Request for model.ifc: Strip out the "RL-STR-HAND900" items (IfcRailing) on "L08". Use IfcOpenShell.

First a look at what the model holds.

```python
import ifcopenshell
import ifcopenshell.util.element

model = ifcopenshell.open("model.ifc")
print(model.schema)
storey = next(s for s in model.by_type("IfcBuildingStorey") if s.Name == "L08")
railings = [e for e in ifcopenshell.util.element.get_decomposition(storey) if e.is_a("IfcRailing")]
seen = {}
for e in railings:
    element_type = ifcopenshell.util.element.get_type(e)
    name = element_type.Name if element_type not in (None, e) else None
    seen[name] = seen.get(name, 0) + 1
for name, count in sorted(seen.items(), key=str):
    print(count, "x", name)
```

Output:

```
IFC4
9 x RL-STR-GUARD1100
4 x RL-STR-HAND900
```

```python
import ifcopenshell
import ifcopenshell.api.root
import ifcopenshell.util.element

model = ifcopenshell.open("model.ifc")

storey = next(s for s in model.by_type("IfcBuildingStorey") if s.Name == "L08")
railings = [e for e in ifcopenshell.util.element.get_decomposition(storey) if e.is_a("IfcRailing")]
targets = [e for e in railings if (t := ifcopenshell.util.element.get_type(e)) not in (None, e) and t.Name == "RL-STR-HAND900"]

for e in targets:
    ifcopenshell.api.root.remove_product(model, product=e)
print(len(targets), "removed")

model.write("model_v2.ifc")
```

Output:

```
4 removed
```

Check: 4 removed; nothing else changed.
